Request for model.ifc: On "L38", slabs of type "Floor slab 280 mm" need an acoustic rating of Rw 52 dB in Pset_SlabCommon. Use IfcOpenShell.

First a look at what the model holds.

```python
import ifcopenshell
import ifcopenshell.util.element

model = ifcopenshell.open("model.ifc")
print(model.schema)
storey = next(s for s in model.by_type("IfcBuildingStorey") if s.Name == "L38")
slabs = [e for e in ifcopenshell.util.element.get_decomposition(storey) if e.is_a("IfcSlab")]
seen = {}
for e in slabs:
    element_type = ifcopenshell.util.element.get_type(e)
    key = (element_type.Name if element_type != e and element_type else None, ifcopenshell.util.element.get_pset(e, "Pset_SlabCommon", "AcousticRating"))
    seen[key] = seen.get(key, 0) + 1
for (name, value), count in sorted(seen.items(), key=str):
    print(count, "x", name, "|", value)
```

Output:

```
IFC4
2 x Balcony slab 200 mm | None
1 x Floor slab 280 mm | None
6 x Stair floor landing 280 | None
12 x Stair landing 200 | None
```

```python
import ifcopenshell
import ifcopenshell.api.pset
import ifcopenshell.util.element

model = ifcopenshell.open("model.ifc")

storey = next(s for s in model.by_type("IfcBuildingStorey") if s.Name == "L38")
slabs = [e for e in ifcopenshell.util.element.get_decomposition(storey) if e.is_a("IfcSlab")]

count = 0
for e in slabs:
    element_type = ifcopenshell.util.element.get_type(e)
    if element_type in (None, e) or element_type.Name != "Floor slab 280 mm":
        continue
    found = ifcopenshell.util.element.get_pset(e, "Pset_SlabCommon", should_inherit=False)
    if found:
        pset = model.by_id(found["id"])
        if len(ifcopenshell.util.element.get_elements_by_pset(pset)) > 1:
            pset = ifcopenshell.api.pset.unshare_pset(model, products=[e], pset=pset)[0]
    else:
        pset = ifcopenshell.api.pset.add_pset(model, product=e, name="Pset_SlabCommon")
    ifcopenshell.api.pset.edit_pset(model, pset=pset, properties={"AcousticRating": "Rw 52 dB"})
    count += 1

print(count, "slabs updated")

model.write("model_updated.ifc")
```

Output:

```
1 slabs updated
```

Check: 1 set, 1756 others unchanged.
